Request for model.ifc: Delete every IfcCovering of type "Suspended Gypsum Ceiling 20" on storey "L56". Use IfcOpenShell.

First a look at what the model holds.

```python
import ifcopenshell
import ifcopenshell.util.element

model = ifcopenshell.open("model.ifc")
print(model.schema)
storey = next(s for s in model.by_type("IfcBuildingStorey") if s.Name == "L56")
coverings = [e for e in ifcopenshell.util.element.get_decomposition(storey) if e.is_a("IfcCovering")]
seen = {}
for e in coverings:
    element_type = ifcopenshell.util.element.get_type(e)
    name = element_type.Name if element_type not in (None, e) else None
    seen[name] = seen.get(name, 0) + 1
for name, count in sorted(seen.items(), key=str):
    print(count, "x", name)
```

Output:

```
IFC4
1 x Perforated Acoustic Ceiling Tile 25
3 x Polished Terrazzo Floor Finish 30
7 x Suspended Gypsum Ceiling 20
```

```python
import ifcopenshell
import ifcopenshell.api.root
import ifcopenshell.util.element

model = ifcopenshell.open("model.ifc")

storey = next(s for s in model.by_type("IfcBuildingStorey") if s.Name == "L56")
coverings = [e for e in ifcopenshell.util.element.get_decomposition(storey) if e.is_a("IfcCovering")]
targets = [e for e in coverings if (t := ifcopenshell.util.element.get_type(e)) not in (None, e) and t.Name == "Suspended Gypsum Ceiling 20"]

for e in targets:
    ifcopenshell.api.root.remove_product(model, product=e)
print(len(targets), "removed")

model.write("model_rev.ifc")
```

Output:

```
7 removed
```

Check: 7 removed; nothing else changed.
